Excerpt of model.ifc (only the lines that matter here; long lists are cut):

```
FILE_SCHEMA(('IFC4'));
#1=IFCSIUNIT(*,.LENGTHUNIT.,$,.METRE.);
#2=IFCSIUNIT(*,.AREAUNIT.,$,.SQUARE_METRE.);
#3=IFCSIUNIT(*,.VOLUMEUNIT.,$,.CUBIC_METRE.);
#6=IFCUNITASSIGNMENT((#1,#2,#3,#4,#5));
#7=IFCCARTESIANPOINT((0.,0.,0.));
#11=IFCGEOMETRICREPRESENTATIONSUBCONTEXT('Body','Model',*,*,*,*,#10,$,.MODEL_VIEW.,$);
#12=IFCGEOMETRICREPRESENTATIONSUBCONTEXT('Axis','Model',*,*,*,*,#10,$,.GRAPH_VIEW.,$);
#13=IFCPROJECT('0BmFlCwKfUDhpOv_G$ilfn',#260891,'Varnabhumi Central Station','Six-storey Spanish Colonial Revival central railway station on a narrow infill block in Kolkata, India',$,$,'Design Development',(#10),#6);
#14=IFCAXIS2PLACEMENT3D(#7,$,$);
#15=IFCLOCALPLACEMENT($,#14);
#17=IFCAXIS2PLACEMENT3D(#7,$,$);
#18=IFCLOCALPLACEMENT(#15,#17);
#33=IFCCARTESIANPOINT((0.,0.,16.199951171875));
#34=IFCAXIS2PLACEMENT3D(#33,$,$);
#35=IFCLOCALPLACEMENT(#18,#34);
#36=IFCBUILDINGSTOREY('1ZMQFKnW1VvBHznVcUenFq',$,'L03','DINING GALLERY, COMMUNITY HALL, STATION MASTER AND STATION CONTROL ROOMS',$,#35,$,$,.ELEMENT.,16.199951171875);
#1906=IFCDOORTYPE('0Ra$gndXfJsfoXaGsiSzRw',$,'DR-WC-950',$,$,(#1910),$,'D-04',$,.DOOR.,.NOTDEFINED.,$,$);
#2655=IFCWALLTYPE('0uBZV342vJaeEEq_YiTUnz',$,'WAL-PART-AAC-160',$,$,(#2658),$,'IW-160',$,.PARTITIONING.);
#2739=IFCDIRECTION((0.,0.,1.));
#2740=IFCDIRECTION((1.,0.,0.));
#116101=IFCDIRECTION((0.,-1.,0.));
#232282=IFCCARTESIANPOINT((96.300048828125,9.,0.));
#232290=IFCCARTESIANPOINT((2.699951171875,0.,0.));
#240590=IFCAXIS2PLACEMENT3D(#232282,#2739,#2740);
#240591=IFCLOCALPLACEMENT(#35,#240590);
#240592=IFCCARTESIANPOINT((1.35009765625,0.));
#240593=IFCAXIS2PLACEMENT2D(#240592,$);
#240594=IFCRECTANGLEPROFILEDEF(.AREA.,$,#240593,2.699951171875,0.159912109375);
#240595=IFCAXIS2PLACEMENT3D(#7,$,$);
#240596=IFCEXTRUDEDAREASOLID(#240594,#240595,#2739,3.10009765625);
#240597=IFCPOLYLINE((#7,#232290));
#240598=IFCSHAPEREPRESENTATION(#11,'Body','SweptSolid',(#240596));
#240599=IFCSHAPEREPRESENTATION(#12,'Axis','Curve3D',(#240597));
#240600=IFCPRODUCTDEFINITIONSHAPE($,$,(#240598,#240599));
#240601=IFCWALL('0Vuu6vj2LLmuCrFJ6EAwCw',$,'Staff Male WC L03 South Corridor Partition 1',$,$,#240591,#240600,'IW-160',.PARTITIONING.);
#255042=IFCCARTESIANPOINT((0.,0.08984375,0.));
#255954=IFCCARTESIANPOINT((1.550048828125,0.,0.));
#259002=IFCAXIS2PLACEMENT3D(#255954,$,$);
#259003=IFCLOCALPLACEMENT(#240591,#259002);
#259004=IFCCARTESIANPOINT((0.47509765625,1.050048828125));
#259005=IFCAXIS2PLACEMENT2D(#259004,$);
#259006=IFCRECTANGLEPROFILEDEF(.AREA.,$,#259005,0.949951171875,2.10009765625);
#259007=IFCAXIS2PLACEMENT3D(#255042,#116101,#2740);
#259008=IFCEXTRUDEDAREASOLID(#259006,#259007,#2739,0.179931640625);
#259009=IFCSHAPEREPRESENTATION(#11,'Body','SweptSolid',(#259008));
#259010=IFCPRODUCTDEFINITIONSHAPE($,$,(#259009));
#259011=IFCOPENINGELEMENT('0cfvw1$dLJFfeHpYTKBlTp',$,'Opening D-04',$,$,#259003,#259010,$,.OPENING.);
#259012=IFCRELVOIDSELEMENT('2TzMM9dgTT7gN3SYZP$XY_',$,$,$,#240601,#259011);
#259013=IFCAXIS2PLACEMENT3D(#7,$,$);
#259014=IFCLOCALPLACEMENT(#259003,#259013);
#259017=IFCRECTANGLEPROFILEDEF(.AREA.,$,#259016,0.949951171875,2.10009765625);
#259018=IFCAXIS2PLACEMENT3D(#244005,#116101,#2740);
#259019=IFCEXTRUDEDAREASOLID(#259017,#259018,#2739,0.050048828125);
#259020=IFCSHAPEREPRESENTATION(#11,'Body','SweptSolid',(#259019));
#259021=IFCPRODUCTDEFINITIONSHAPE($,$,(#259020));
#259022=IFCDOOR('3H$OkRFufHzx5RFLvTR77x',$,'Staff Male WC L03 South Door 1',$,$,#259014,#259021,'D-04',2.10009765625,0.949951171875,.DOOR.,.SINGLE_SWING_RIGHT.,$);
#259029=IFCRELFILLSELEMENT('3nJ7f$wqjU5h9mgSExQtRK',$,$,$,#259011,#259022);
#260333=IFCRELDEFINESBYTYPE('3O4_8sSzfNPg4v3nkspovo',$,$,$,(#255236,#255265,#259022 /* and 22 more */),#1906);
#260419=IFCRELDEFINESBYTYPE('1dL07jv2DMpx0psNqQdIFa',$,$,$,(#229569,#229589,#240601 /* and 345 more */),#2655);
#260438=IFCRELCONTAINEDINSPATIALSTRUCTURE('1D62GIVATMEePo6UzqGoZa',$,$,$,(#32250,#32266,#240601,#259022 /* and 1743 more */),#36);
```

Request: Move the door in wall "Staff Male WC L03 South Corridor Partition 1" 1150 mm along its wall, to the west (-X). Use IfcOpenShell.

```python
import ifcopenshell
import ifcopenshell.api.geometry
import ifcopenshell.util.placement
import ifcopenshell.util.unit

model = ifcopenshell.open("model.ifc")
unit_scale = ifcopenshell.util.unit.calculate_unit_scale(model)

door = model.by_id(259022)
opening = door.FillsVoids[0].RelatingOpeningElement
wall = opening.VoidsElements[0].RelatingBuildingElement

wall_matrix = ifcopenshell.util.placement.get_local_placement(wall.ObjectPlacement)
shift = wall_matrix[:3, 0] * -1.15 / unit_scale
before = ifcopenshell.util.placement.get_local_placement(door.ObjectPlacement)[:3, 3].copy()

# The door is placed relative to its opening, so it follows when the opening moves.
matrix = ifcopenshell.util.placement.get_local_placement(opening.ObjectPlacement)
matrix[:3, 3] += shift
ifcopenshell.api.geometry.edit_object_placement(
    model, product=opening, matrix=matrix, is_si=False, should_transform_children=True
)

after = ifcopenshell.util.placement.get_local_placement(door.ObjectPlacement)[:3, 3]
print("door moved by", (after - before).round(3) + 0.0)

model.write("model-out.ifc")
```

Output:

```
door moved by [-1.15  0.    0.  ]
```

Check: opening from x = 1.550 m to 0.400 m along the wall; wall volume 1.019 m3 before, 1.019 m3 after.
